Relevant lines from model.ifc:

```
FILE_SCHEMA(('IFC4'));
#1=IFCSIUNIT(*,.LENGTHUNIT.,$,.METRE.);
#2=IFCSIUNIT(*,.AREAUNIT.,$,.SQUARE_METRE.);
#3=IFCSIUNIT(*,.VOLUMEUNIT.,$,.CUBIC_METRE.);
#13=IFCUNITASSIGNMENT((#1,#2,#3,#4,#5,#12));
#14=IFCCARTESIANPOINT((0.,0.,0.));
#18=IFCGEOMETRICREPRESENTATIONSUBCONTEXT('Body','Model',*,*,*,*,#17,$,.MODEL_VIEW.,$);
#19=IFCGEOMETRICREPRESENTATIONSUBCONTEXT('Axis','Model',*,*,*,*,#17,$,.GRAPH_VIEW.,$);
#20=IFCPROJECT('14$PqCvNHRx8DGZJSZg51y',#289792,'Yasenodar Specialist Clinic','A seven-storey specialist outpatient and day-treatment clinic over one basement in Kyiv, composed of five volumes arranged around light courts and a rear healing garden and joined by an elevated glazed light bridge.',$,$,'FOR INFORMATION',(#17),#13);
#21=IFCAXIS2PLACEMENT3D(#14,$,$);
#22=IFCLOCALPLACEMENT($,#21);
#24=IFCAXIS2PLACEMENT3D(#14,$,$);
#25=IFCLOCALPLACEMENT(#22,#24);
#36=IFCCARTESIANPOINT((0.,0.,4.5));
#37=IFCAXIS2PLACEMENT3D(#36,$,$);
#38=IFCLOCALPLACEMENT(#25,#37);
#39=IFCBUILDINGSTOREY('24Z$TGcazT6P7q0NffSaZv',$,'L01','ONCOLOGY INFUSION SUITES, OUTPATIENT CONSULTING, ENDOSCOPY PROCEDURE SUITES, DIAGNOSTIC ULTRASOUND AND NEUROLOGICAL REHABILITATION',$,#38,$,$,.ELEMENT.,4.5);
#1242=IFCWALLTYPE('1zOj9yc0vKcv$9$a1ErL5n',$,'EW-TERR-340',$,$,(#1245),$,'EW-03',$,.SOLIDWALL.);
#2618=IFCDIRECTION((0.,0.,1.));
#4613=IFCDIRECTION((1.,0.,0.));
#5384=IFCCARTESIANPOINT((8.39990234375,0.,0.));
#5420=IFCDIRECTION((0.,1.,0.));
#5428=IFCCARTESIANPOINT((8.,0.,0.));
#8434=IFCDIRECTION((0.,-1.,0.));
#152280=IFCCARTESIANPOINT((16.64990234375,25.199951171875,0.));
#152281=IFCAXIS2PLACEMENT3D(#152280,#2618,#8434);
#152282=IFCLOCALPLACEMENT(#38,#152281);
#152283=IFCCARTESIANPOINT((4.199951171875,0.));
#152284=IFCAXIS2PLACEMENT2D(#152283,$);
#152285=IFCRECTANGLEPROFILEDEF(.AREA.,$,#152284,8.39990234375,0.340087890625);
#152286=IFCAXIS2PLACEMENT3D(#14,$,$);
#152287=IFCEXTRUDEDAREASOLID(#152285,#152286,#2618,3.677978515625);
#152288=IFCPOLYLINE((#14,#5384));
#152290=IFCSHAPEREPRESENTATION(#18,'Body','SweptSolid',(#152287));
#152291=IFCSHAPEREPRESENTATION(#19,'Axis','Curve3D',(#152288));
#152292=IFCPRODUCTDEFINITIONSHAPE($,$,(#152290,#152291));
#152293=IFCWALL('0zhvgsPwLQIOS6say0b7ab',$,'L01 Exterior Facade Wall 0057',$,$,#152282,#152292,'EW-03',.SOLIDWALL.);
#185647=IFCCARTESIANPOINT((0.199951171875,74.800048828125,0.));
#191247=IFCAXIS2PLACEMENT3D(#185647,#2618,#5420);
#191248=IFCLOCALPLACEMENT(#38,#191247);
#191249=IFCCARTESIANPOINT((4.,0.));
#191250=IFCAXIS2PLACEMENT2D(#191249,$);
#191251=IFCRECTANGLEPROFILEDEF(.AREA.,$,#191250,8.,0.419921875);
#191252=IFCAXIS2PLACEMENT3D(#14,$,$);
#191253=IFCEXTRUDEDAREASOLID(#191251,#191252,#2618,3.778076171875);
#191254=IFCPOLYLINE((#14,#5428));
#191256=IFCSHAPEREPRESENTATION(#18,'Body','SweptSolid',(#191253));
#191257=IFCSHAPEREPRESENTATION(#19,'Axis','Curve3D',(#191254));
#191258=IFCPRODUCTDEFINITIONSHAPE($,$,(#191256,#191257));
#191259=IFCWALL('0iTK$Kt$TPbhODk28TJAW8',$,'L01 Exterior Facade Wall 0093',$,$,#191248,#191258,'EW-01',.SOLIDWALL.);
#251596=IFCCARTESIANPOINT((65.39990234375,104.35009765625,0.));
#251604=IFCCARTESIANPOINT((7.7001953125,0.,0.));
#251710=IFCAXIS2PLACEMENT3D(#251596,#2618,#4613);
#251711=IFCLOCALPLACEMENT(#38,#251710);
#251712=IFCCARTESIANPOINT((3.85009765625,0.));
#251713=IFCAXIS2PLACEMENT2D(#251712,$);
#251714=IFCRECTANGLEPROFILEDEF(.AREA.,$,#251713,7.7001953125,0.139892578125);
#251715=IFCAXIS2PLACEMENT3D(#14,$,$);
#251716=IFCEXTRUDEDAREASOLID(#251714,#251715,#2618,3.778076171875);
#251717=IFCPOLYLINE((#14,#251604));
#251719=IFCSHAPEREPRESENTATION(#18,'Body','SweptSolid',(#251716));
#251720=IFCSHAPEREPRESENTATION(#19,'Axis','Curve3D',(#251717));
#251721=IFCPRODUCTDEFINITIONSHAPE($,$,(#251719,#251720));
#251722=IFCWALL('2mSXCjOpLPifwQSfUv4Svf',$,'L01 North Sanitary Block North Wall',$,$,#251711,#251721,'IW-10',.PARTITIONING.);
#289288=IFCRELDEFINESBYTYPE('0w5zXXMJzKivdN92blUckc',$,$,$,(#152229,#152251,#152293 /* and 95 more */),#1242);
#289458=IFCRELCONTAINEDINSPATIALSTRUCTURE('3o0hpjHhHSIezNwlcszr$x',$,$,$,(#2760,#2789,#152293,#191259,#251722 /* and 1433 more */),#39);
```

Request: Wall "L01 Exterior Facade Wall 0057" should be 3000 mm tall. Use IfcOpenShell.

```python
import ifcopenshell
import ifcopenshell.geom
import ifcopenshell.util.representation
import ifcopenshell.util.shape

model = ifcopenshell.open("model.ifc")
settings = ifcopenshell.geom.settings()


def volume(element):
    """Net volume in cubic metres, openings subtracted."""
    shape = ifcopenshell.geom.create_shape(settings, element)
    return ifcopenshell.util.shape.get_volume(shape.geometry)


wall = model.by_guid("0zhvgsPwLQIOS6say0b7ab")
before = volume(wall)

body = ifcopenshell.util.representation.get_representation(wall, "Model", "Body")
solid = body.Items[0]
old_height = solid.Depth
solid.Depth = 3.0
after = volume(wall)

print(f"height {old_height:g} -> {solid.Depth:g}, volume {before:.3f} -> {after:.3f} m3")

model.write("model_rev.ifc")
```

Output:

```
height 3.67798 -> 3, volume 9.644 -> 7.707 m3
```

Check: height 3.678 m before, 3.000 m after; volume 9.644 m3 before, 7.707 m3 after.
